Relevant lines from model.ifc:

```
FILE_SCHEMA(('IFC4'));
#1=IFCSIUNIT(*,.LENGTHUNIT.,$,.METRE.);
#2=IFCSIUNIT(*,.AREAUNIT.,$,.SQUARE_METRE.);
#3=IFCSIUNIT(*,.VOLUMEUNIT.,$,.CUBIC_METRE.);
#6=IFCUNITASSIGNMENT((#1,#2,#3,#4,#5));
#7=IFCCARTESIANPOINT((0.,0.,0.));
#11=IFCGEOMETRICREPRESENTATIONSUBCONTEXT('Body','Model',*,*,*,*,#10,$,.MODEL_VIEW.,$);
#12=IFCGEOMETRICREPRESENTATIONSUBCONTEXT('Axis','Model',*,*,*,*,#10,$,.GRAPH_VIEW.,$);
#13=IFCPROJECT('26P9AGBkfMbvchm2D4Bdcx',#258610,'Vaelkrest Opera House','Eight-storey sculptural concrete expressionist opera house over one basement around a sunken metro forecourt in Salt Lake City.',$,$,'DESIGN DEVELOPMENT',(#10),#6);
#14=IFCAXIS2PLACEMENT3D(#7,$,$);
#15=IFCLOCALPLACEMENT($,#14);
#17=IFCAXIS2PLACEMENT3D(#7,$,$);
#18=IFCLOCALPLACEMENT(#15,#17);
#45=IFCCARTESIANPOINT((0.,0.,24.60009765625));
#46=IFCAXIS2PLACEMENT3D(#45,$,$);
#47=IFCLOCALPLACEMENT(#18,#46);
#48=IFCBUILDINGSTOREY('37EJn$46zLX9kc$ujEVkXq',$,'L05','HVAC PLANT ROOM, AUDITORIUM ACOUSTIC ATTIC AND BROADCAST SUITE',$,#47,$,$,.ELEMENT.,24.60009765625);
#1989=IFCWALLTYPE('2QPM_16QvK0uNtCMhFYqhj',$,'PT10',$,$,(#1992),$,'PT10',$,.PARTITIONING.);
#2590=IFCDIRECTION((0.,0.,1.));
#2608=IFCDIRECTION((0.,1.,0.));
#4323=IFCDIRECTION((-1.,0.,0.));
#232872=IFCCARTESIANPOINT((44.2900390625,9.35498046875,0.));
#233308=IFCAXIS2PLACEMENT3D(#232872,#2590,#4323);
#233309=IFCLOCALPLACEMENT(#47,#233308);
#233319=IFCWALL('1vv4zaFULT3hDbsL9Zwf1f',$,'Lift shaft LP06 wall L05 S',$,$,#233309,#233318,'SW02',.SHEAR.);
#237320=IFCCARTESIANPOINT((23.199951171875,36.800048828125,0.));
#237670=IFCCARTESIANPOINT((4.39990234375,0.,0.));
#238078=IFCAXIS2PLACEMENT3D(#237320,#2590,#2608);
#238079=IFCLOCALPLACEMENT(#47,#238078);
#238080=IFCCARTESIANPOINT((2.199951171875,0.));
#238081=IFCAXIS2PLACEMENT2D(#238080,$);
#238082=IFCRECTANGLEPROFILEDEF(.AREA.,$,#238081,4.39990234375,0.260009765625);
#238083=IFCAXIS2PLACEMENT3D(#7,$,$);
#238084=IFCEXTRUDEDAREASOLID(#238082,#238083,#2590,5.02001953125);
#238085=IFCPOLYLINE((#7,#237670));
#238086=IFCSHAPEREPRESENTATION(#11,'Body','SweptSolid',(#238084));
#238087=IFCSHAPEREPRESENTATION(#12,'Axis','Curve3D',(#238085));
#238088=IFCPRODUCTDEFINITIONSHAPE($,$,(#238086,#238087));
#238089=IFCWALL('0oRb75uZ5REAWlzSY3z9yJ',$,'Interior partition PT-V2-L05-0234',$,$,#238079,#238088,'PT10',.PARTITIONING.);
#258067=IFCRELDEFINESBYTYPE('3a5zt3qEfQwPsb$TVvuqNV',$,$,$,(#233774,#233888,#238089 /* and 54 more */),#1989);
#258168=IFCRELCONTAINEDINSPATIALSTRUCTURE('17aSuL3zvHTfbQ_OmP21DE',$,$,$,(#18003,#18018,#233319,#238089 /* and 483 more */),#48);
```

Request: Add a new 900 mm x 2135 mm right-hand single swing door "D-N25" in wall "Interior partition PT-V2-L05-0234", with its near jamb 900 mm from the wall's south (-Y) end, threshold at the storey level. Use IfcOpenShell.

```python
import numpy as np
import ifcopenshell
import ifcopenshell.api.feature
import ifcopenshell.api.geometry
import ifcopenshell.api.root
import ifcopenshell.api.spatial
import ifcopenshell.geom
import ifcopenshell.util.element
import ifcopenshell.util.placement
import ifcopenshell.util.representation
import ifcopenshell.util.shape
import ifcopenshell.util.unit

model = ifcopenshell.open("model.ifc")
unit_scale = ifcopenshell.util.unit.calculate_unit_scale(model)
settings = ifcopenshell.geom.settings()


def volume(element):
    """Net volume in cubic metres, openings subtracted."""
    shape = ifcopenshell.geom.create_shape(settings, element)
    return ifcopenshell.util.shape.get_volume(shape.geometry)


wall = model.by_guid("0oRb75uZ5REAWlzSY3z9yJ")
storey = ifcopenshell.util.element.get_container(wall, ifc_class="IfcBuildingStorey")
context = ifcopenshell.util.representation.get_context(model, "Model", "Body", "MODEL_VIEW")
before = volume(wall)

width, height, from_end, sill = 0.9, 2.135, 0.9, 0.0  # metres

# The wall runs along its own X axis, and the end named is its -X end.
wall_shape = ifcopenshell.geom.create_shape(settings, wall)
x, y, z = ifcopenshell.util.shape.get_vertices(wall_shape.geometry).T
start = x.min() + from_end
face, thickness = float(y.min()), float(y.max() - y.min())
wall_matrix = ifcopenshell.util.placement.get_local_placement(wall.ObjectPlacement)
level = ifcopenshell.util.placement.get_local_placement(storey.ObjectPlacement)[2, 3]


def in_wall(x, y):
    """Placement at x, y metres in the wall's axes, at sill height."""
    matrix = wall_matrix.copy()
    matrix[:, 3] = wall_matrix @ np.array([x / unit_scale, y / unit_scale, 0.0, 1.0])
    matrix[2, 3] = level + sill / unit_scale
    return matrix


# Opening: a box that overshoots both wall faces by 50 mm.
opening = ifcopenshell.api.root.create_entity(model, ifc_class="IfcOpeningElement", predefined_type="OPENING")
box = ifcopenshell.api.geometry.add_wall_representation(
    model, context=context, length=width, height=height, thickness=thickness + 0.1
)
ifcopenshell.api.geometry.assign_representation(model, product=opening, representation=box)
ifcopenshell.api.geometry.edit_object_placement(model, product=opening, matrix=in_wall(start, face - 0.05), is_si=False)
ifcopenshell.api.feature.add_feature(model, feature=opening, element=wall)

door = ifcopenshell.api.root.create_entity(model, ifc_class="IfcDoor", name="D-N25", predefined_type="DOOR")
door.OverallWidth, door.OverallHeight = width / unit_scale, height / unit_scale
door.OperationType = "SINGLE_SWING_RIGHT"
body = ifcopenshell.api.geometry.add_door_representation(
    model,
    context=context,
    overall_width=door.OverallWidth,
    overall_height=door.OverallHeight,
    operation_type="SINGLE_SWING_RIGHT",
    lining_properties={"LiningDepth": thickness / unit_scale, "ThresholdDepth": thickness / unit_scale},
)
ifcopenshell.api.geometry.assign_representation(model, product=door, representation=body)
ifcopenshell.api.spatial.assign_container(model, products=[door], relating_structure=storey)
ifcopenshell.api.feature.add_filling(model, opening=opening, element=door)

# The lining spans the wall, so the door starts at the wall face.
ifcopenshell.api.geometry.edit_object_placement(model, product=door, matrix=in_wall(start, face), is_si=False)

after = volume(wall)

print(f"wall volume {before:.3f} -> {after:.3f} m3")

model.write("model_v2.ifc")
```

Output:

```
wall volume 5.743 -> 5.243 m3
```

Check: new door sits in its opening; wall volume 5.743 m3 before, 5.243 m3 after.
